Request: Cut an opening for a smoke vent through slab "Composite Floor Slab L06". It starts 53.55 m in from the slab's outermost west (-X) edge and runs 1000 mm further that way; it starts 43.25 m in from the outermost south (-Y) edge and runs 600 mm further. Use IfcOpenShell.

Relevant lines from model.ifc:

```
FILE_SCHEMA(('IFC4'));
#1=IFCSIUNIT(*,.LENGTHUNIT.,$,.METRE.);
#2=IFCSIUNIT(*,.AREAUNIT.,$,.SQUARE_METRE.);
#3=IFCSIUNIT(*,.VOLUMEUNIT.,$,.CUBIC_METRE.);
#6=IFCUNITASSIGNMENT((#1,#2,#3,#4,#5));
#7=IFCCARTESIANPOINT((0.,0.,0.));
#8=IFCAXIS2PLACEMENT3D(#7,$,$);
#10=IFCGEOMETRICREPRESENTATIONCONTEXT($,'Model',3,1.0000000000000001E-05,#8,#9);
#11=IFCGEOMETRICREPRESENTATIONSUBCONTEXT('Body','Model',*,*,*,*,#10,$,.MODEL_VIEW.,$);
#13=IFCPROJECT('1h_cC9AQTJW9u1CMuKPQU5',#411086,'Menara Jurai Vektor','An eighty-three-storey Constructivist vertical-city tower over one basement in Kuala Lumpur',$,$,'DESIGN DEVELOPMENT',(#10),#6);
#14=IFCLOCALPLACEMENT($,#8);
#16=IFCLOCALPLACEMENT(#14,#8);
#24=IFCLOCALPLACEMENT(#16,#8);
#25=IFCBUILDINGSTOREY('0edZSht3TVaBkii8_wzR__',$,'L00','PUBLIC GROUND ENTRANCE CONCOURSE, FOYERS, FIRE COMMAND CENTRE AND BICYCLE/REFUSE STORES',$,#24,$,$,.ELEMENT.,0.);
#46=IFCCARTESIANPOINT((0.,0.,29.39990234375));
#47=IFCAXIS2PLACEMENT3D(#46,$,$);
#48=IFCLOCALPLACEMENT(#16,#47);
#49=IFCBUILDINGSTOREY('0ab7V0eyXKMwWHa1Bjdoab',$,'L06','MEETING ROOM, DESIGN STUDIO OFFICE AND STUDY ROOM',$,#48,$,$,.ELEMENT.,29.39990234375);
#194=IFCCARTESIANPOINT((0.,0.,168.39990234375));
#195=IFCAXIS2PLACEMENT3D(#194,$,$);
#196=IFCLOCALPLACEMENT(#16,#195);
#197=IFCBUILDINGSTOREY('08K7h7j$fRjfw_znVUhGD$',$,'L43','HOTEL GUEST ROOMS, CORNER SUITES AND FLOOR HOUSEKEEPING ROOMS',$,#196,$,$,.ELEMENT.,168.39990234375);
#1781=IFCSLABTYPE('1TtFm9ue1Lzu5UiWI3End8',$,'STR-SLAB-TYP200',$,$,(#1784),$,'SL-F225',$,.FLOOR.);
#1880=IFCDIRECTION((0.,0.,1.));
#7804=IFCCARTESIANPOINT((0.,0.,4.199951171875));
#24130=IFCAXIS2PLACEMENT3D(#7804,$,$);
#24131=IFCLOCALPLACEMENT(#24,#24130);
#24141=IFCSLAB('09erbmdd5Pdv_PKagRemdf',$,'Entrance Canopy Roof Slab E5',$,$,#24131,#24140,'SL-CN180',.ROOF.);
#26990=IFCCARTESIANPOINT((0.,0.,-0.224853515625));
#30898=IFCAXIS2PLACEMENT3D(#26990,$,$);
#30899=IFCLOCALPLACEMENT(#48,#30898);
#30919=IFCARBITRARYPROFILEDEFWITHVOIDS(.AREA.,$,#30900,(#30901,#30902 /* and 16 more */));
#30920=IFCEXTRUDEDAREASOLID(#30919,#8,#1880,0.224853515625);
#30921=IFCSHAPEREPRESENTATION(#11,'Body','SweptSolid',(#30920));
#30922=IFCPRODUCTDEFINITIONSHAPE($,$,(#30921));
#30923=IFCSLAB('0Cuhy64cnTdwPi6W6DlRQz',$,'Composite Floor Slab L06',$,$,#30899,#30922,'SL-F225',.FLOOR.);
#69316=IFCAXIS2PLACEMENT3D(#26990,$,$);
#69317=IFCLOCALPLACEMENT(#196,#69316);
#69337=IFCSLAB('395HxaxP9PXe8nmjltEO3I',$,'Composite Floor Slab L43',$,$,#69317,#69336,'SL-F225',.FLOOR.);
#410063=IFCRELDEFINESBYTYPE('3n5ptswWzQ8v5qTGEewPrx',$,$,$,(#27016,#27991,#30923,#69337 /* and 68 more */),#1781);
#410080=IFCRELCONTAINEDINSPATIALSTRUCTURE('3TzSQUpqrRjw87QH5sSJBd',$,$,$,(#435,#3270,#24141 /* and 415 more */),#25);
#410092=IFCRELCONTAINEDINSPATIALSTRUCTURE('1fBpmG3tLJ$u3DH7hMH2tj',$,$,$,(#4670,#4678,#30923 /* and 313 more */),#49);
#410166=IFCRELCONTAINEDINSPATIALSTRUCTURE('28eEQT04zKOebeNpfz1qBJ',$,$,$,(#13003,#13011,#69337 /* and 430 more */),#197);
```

```python
import numpy as np
import ifcopenshell
import ifcopenshell.api.feature
import ifcopenshell.api.geometry
import ifcopenshell.api.root
import ifcopenshell.geom
import ifcopenshell.util.placement
import ifcopenshell.util.representation
import ifcopenshell.util.shape
import ifcopenshell.util.unit

model = ifcopenshell.open("model.ifc")
unit_scale = ifcopenshell.util.unit.calculate_unit_scale(model)
settings = ifcopenshell.geom.settings()


def volume(element):
    """Net volume in cubic metres, openings subtracted."""
    shape = ifcopenshell.geom.create_shape(settings, element)
    return ifcopenshell.util.shape.get_volume(shape.geometry)


slab = model.by_id(30923)
before = volume(slab)

# Extent in the slab's own axes, in metres. The edges named are its -X and -Y sides.
slab_shape = ifcopenshell.geom.create_shape(settings, slab)
vertices = ifcopenshell.util.shape.get_vertices(slab_shape.geometry)
x_min, y_min, bottom = vertices.min(axis=0)
top = vertices[:, 2].max()

opening = ifcopenshell.api.root.create_entity(model, ifc_class="IfcOpeningElement", name="Smoke vent opening", predefined_type="OPENING")
context = ifcopenshell.util.representation.get_context(model, "Model", "Body", "MODEL_VIEW")
width, depth = 1, 0.6
outline = [(0.0, 0.0), (width, 0.0), (width, depth), (0.0, depth), (0.0, 0.0)]
# Overshoot both faces by 50 mm so the cut is clean.
shape = ifcopenshell.api.geometry.add_slab_representation(
    model, context=context, depth=top - bottom + 0.1, polyline=outline
)
ifcopenshell.api.geometry.assign_representation(model, product=opening, representation=shape)

matrix = ifcopenshell.util.placement.get_local_placement(slab.ObjectPlacement)
matrix[:, 3] = matrix @ np.append(np.array([x_min + 53.55, y_min + 43.25, bottom - 0.05]) / unit_scale, 1.0)
ifcopenshell.api.geometry.edit_object_placement(model, product=opening, matrix=matrix, is_si=False)
ifcopenshell.api.feature.add_feature(model, feature=opening, element=slab)

after = volume(slab)

print(f"slab volume {before:.3f} -> {after:.3f} m3")

model.write("model-out.ifc")
```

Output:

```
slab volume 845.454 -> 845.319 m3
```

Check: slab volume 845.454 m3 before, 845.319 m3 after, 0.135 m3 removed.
